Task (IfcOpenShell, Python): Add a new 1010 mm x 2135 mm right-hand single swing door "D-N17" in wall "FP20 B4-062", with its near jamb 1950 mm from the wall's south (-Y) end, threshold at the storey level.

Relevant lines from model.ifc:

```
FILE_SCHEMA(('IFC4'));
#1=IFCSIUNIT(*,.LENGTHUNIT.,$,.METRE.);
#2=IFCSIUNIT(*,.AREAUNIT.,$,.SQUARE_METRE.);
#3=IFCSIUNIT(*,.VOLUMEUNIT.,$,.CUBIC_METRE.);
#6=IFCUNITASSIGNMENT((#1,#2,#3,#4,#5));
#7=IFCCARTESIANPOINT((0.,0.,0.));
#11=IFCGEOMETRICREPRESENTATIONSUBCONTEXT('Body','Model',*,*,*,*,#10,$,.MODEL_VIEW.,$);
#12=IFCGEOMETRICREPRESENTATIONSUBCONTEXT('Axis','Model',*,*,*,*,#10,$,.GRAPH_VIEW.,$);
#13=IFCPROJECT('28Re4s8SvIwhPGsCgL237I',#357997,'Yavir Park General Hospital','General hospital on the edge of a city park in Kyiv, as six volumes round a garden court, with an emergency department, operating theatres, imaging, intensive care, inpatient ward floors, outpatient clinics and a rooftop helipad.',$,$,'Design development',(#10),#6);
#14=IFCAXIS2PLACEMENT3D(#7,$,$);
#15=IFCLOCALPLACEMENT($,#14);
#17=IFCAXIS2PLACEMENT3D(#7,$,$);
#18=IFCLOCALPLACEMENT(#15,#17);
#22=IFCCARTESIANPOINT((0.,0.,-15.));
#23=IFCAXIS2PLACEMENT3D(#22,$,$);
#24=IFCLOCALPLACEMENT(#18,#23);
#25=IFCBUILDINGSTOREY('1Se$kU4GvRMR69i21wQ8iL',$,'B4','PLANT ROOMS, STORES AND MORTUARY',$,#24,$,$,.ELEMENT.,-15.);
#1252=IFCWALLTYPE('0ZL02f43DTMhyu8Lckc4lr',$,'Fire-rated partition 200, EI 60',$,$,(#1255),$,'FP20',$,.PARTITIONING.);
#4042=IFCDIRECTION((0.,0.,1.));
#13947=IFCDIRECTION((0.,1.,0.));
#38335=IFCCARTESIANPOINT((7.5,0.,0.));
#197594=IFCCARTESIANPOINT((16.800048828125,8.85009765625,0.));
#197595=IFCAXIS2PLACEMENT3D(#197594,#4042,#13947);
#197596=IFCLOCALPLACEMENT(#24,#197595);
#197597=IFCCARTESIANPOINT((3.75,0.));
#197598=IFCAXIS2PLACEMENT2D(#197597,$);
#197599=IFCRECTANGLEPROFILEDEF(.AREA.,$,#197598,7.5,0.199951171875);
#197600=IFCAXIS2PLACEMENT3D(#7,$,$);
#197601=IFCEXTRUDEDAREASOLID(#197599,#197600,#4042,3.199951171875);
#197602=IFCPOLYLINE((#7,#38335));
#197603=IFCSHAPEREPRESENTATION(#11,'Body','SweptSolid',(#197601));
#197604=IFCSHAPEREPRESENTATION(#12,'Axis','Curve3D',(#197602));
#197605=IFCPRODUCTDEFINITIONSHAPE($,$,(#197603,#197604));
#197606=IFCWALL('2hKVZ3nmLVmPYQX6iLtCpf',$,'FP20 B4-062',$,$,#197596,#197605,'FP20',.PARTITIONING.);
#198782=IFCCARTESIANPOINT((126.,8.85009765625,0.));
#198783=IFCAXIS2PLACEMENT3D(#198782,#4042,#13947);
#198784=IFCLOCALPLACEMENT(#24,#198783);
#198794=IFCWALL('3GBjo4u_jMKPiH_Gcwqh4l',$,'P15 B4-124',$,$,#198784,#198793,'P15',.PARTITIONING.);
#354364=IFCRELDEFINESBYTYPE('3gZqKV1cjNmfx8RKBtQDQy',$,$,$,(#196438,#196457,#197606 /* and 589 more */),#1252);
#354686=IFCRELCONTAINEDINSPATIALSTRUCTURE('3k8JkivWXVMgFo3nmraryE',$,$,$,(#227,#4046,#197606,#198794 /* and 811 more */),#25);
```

```python
import numpy as np
import ifcopenshell
import ifcopenshell.api.feature
import ifcopenshell.api.geometry
import ifcopenshell.api.root
import ifcopenshell.api.spatial
import ifcopenshell.geom
import ifcopenshell.util.element
import ifcopenshell.util.placement
import ifcopenshell.util.representation
import ifcopenshell.util.shape
import ifcopenshell.util.unit

model = ifcopenshell.open("model.ifc")
unit_scale = ifcopenshell.util.unit.calculate_unit_scale(model)
settings = ifcopenshell.geom.settings()


def volume(element):
    """Net volume in cubic metres, openings subtracted."""
    shape = ifcopenshell.geom.create_shape(settings, element)
    return ifcopenshell.util.shape.get_volume(shape.geometry)


wall = model.by_guid("2hKVZ3nmLVmPYQX6iLtCpf")
storey = ifcopenshell.util.element.get_container(wall, ifc_class="IfcBuildingStorey")
context = ifcopenshell.util.representation.get_context(model, "Model", "Body", "MODEL_VIEW")
before = volume(wall)

width, height, from_end, sill = 1.01, 2.135, 1.95, 0.0  # metres

# The wall runs along its own X axis, and the end named is its -X end.
wall_shape = ifcopenshell.geom.create_shape(settings, wall)
x, y, z = ifcopenshell.util.shape.get_vertices(wall_shape.geometry).T
start = x.min() + from_end
face, thickness = float(y.min()), float(y.max() - y.min())
wall_matrix = ifcopenshell.util.placement.get_local_placement(wall.ObjectPlacement)
level = ifcopenshell.util.placement.get_local_placement(storey.ObjectPlacement)[2, 3]


def in_wall(x, y):
    """Placement at x, y metres in the wall's axes, at sill height."""
    matrix = wall_matrix.copy()
    matrix[:, 3] = wall_matrix @ np.array([x / unit_scale, y / unit_scale, 0.0, 1.0])
    matrix[2, 3] = level + sill / unit_scale
    return matrix


# Opening: a box that overshoots both wall faces by 50 mm.
opening = ifcopenshell.api.root.create_entity(model, ifc_class="IfcOpeningElement", predefined_type="OPENING")
box = ifcopenshell.api.geometry.add_wall_representation(
    model, context=context, length=width, height=height, thickness=thickness + 0.1
)
ifcopenshell.api.geometry.assign_representation(model, product=opening, representation=box)
ifcopenshell.api.geometry.edit_object_placement(model, product=opening, matrix=in_wall(start, face - 0.05), is_si=False)
ifcopenshell.api.feature.add_feature(model, feature=opening, element=wall)

door = ifcopenshell.api.root.create_entity(model, ifc_class="IfcDoor", name="D-N17", predefined_type="DOOR")
door.OverallWidth, door.OverallHeight = width / unit_scale, height / unit_scale
door.OperationType = "SINGLE_SWING_RIGHT"
body = ifcopenshell.api.geometry.add_door_representation(
    model,
    context=context,
    overall_width=door.OverallWidth,
    overall_height=door.OverallHeight,
    operation_type="SINGLE_SWING_RIGHT",
    lining_properties={"LiningDepth": thickness / unit_scale, "ThresholdDepth": thickness / unit_scale},
)
ifcopenshell.api.geometry.assign_representation(model, product=door, representation=body)
ifcopenshell.api.spatial.assign_container(model, products=[door], relating_structure=storey)
ifcopenshell.api.feature.add_filling(model, opening=opening, element=door)

# The lining spans the wall, so the door starts at the wall face.
ifcopenshell.api.geometry.edit_object_placement(model, product=door, matrix=in_wall(start, face), is_si=False)

after = volume(wall)

print(f"wall volume {before:.3f} -> {after:.3f} m3")

model.write("model_updated.ifc")
```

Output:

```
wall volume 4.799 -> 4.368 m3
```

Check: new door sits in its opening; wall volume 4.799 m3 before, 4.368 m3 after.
